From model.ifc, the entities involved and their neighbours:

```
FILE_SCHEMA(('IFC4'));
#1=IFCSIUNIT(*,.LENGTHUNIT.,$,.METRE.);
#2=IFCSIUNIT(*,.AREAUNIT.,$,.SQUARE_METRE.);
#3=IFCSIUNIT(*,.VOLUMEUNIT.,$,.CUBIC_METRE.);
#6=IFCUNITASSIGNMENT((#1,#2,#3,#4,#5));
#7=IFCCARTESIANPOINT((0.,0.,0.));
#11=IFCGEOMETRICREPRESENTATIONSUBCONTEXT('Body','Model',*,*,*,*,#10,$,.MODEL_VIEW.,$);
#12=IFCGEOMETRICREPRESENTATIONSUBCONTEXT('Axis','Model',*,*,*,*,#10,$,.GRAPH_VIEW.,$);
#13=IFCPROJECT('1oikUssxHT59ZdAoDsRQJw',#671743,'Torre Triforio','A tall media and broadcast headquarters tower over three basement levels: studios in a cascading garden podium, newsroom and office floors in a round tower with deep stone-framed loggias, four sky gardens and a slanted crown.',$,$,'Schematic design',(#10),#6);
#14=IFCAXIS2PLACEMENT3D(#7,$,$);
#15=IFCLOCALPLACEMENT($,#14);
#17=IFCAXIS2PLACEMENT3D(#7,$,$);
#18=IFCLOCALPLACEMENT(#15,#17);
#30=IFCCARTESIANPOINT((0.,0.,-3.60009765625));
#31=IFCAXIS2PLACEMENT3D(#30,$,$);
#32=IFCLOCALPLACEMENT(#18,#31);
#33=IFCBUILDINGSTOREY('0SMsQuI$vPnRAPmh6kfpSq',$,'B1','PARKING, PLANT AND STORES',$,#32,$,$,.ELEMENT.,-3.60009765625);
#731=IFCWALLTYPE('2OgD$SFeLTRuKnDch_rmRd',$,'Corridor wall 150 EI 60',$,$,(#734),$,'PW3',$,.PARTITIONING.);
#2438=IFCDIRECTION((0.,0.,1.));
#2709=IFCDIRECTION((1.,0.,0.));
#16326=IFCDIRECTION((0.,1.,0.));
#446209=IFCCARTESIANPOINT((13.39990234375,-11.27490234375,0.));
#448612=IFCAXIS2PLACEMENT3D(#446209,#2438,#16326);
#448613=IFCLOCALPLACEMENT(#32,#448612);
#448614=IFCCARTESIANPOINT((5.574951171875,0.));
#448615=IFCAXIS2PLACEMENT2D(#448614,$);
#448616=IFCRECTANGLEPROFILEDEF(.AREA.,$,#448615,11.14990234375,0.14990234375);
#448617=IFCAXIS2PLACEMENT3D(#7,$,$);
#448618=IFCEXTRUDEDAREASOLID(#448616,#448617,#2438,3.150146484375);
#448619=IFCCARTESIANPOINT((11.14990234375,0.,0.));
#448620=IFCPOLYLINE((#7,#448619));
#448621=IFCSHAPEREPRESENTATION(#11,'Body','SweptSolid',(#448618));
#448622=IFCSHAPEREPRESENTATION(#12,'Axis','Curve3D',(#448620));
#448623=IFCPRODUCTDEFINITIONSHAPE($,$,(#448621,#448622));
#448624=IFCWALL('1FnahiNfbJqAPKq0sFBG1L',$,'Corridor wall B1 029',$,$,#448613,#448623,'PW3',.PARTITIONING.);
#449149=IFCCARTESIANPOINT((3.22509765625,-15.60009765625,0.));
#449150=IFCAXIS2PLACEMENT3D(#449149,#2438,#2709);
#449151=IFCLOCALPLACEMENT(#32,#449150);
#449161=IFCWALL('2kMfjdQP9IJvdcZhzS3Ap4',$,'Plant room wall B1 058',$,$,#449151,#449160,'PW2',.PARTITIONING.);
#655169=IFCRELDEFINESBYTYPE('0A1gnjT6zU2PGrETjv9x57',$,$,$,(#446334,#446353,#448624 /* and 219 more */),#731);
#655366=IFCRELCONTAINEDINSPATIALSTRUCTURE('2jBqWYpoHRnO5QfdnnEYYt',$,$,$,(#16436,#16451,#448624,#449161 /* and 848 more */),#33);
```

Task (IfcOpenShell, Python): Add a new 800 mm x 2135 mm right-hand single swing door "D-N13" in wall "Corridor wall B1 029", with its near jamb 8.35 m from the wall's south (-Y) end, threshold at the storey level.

```python
import numpy as np
import ifcopenshell
import ifcopenshell.api.feature
import ifcopenshell.api.geometry
import ifcopenshell.api.root
import ifcopenshell.api.spatial
import ifcopenshell.geom
import ifcopenshell.util.element
import ifcopenshell.util.placement
import ifcopenshell.util.representation
import ifcopenshell.util.shape
import ifcopenshell.util.unit

model = ifcopenshell.open("model.ifc")
unit_scale = ifcopenshell.util.unit.calculate_unit_scale(model)
settings = ifcopenshell.geom.settings()


def volume(element):
    """Net volume in cubic metres, openings subtracted."""
    shape = ifcopenshell.geom.create_shape(settings, element)
    return ifcopenshell.util.shape.get_volume(shape.geometry)


wall = model.by_guid("1FnahiNfbJqAPKq0sFBG1L")
storey = ifcopenshell.util.element.get_container(wall, ifc_class="IfcBuildingStorey")
context = ifcopenshell.util.representation.get_context(model, "Model", "Body", "MODEL_VIEW")
before = volume(wall)

width, height, from_end, sill = 0.8, 2.135, 8.35, 0.0  # metres

# The wall runs along its own X axis, and the end named is its -X end.
wall_shape = ifcopenshell.geom.create_shape(settings, wall)
x, y, z = ifcopenshell.util.shape.get_vertices(wall_shape.geometry).T
start = x.min() + from_end
face, thickness = float(y.min()), float(y.max() - y.min())
wall_matrix = ifcopenshell.util.placement.get_local_placement(wall.ObjectPlacement)
level = ifcopenshell.util.placement.get_local_placement(storey.ObjectPlacement)[2, 3]


def in_wall(x, y):
    """Placement at x, y metres in the wall's axes, at sill height."""
    matrix = wall_matrix.copy()
    matrix[:, 3] = wall_matrix @ np.array([x / unit_scale, y / unit_scale, 0.0, 1.0])
    matrix[2, 3] = level + sill / unit_scale
    return matrix


# Opening: a box that overshoots both wall faces by 50 mm.
opening = ifcopenshell.api.root.create_entity(model, ifc_class="IfcOpeningElement", predefined_type="OPENING")
box = ifcopenshell.api.geometry.add_wall_representation(
    model, context=context, length=width, height=height, thickness=thickness + 0.1
)
ifcopenshell.api.geometry.assign_representation(model, product=opening, representation=box)
ifcopenshell.api.geometry.edit_object_placement(model, product=opening, matrix=in_wall(start, face - 0.05), is_si=False)
ifcopenshell.api.feature.add_feature(model, feature=opening, element=wall)

door = ifcopenshell.api.root.create_entity(model, ifc_class="IfcDoor", name="D-N13", predefined_type="DOOR")
door.OverallWidth, door.OverallHeight = width / unit_scale, height / unit_scale
door.OperationType = "SINGLE_SWING_RIGHT"
body = ifcopenshell.api.geometry.add_door_representation(
    model,
    context=context,
    overall_width=door.OverallWidth,
    overall_height=door.OverallHeight,
    operation_type="SINGLE_SWING_RIGHT",
    lining_properties={"LiningDepth": thickness / unit_scale, "ThresholdDepth": thickness / unit_scale},
)
ifcopenshell.api.geometry.assign_representation(model, product=door, representation=body)
ifcopenshell.api.spatial.assign_container(model, products=[door], relating_structure=storey)
ifcopenshell.api.feature.add_filling(model, opening=opening, element=door)

# The lining spans the wall, so the door starts at the wall face.
ifcopenshell.api.geometry.edit_object_placement(model, product=door, matrix=in_wall(start, face), is_si=False)

after = volume(wall)

print(f"wall volume {before:.3f} -> {after:.3f} m3")

model.write("model_updated.ifc")
```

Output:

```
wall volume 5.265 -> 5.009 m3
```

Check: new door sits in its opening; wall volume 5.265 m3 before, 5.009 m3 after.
